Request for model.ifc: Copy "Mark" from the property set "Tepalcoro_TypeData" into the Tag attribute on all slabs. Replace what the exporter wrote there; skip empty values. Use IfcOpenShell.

First a look at what the model holds.

```python
import ifcopenshell
import ifcopenshell.util.element

model = ifcopenshell.open("model.ifc")
print(model.schema)
slabs = model.by_type("IfcSlab")
print(len(slabs), "slabs")
for e in slabs[:8]:
    source = ifcopenshell.util.element.get_pset(e, "Tepalcoro_TypeData", "Mark")
    target = e.Tag
    print(e.id(), repr(source), repr(target), sep=" | ")
```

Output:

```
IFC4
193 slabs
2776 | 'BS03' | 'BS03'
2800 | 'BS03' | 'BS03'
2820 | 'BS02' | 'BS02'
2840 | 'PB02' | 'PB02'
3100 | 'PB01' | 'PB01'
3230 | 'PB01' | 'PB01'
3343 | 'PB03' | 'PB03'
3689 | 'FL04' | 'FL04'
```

```python
import ifcopenshell
import ifcopenshell.util.element

model = ifcopenshell.open("model.ifc")

count = 0
for e in model.by_type("IfcSlab"):
    value = ifcopenshell.util.element.get_pset(e, "Tepalcoro_TypeData", "Mark")
    current = e.Tag
    if not value or not value.strip() or current == value:
        continue
    e.Tag = value
    count += 1

print(count, "slabs updated")

model.write("model_updated.ifc")
```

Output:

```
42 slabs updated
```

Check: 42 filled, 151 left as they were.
